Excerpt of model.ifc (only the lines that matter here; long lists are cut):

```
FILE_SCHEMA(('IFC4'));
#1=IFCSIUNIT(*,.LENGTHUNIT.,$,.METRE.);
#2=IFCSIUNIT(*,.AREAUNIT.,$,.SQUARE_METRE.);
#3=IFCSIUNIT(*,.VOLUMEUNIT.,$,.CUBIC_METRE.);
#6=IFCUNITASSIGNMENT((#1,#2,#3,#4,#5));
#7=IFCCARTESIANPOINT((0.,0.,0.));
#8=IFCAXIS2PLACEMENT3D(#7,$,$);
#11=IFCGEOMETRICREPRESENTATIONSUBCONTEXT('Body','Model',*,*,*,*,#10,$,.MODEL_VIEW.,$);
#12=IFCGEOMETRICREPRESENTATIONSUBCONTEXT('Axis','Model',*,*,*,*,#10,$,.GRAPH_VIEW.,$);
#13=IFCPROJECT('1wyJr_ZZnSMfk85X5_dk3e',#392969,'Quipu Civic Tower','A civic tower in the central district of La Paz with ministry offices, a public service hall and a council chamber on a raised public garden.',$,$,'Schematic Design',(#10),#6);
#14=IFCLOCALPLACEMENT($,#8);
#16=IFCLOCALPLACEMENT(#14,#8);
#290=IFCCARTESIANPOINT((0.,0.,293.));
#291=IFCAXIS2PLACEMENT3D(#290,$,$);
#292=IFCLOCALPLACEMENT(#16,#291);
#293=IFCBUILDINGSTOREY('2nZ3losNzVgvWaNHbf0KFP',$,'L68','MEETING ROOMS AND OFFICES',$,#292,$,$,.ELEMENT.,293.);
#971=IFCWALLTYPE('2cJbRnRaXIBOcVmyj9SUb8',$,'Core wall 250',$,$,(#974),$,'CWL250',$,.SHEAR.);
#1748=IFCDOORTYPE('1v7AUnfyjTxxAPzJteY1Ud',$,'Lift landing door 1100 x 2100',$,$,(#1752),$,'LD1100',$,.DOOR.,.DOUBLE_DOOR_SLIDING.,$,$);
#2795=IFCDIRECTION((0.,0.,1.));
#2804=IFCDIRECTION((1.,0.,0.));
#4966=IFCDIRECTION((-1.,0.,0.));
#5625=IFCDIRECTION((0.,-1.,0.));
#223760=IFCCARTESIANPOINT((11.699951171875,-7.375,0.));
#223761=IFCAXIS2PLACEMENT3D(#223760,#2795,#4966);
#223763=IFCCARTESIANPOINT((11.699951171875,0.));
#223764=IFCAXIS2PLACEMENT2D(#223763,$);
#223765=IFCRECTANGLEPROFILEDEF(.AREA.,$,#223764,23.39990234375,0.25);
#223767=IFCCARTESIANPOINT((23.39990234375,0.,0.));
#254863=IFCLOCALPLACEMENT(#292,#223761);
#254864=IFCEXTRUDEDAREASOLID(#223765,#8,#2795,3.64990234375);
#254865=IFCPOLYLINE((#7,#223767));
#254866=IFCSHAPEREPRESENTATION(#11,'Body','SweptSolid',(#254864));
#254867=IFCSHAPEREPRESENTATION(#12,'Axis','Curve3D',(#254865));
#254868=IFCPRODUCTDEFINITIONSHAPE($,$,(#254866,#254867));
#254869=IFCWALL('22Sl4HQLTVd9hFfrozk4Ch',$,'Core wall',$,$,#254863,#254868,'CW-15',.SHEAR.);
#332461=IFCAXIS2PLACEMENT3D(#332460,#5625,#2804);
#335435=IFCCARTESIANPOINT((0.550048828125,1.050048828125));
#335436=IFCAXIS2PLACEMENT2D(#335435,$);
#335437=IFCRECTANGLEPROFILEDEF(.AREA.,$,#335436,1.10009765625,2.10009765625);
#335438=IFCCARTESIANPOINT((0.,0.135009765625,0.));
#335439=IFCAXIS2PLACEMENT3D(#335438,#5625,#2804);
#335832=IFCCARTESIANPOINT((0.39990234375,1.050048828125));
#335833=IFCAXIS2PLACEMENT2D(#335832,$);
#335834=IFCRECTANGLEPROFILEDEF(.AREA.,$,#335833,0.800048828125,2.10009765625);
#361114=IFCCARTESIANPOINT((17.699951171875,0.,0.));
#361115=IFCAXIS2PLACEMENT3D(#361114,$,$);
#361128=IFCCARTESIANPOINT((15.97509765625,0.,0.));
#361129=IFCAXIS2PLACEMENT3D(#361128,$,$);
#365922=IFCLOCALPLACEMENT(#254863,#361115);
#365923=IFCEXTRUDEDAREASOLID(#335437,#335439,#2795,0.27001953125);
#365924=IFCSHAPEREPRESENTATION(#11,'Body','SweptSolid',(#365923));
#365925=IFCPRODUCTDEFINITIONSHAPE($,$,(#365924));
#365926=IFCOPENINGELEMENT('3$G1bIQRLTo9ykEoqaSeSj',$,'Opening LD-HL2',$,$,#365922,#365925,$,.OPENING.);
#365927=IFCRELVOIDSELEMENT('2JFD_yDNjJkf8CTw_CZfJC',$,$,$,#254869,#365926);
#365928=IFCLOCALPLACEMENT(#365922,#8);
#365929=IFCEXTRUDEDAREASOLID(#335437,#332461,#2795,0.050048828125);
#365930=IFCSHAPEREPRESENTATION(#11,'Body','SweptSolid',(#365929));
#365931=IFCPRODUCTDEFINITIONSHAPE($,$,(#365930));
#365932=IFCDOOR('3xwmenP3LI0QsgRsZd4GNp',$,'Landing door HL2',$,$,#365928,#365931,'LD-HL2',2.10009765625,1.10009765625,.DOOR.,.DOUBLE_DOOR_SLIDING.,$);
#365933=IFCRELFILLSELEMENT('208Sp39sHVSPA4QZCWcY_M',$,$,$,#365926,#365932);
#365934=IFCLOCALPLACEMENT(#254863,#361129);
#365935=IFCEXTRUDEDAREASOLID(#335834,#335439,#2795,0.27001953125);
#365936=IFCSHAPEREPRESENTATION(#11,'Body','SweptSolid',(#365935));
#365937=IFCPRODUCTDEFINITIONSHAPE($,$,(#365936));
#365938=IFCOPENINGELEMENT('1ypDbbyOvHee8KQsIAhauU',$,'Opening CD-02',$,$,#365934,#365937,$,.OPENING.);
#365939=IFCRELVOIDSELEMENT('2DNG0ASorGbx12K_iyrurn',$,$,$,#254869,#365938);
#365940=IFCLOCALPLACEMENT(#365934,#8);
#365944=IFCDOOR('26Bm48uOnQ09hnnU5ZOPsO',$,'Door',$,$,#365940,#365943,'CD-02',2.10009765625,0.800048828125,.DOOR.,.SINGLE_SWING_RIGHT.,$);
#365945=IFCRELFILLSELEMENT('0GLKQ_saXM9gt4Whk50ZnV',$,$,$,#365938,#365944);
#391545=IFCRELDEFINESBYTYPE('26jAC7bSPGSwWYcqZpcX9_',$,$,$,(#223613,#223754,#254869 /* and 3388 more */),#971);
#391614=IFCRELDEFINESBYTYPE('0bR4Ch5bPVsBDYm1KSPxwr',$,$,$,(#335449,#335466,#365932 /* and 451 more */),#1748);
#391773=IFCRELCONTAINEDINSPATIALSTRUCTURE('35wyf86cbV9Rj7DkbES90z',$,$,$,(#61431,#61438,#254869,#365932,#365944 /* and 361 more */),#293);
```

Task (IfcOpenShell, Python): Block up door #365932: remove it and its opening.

```python
import ifcopenshell
import ifcopenshell.api.feature
import ifcopenshell.api.root
import ifcopenshell.geom
import ifcopenshell.util.shape

model = ifcopenshell.open("model.ifc")
settings = ifcopenshell.geom.settings()


def volume(element):
    """Net volume in cubic metres, openings subtracted."""
    shape = ifcopenshell.geom.create_shape(settings, element)
    return ifcopenshell.util.shape.get_volume(shape.geometry)


door = model.by_guid("3xwmenP3LI0QsgRsZd4GNp")
opening = door.FillsVoids[0].RelatingOpeningElement
wall = opening.VoidsElements[0].RelatingBuildingElement
before = volume(wall)

ifcopenshell.api.root.remove_product(model, product=door)
ifcopenshell.api.feature.remove_feature(model, feature=opening)

after = volume(wall)

print(f"wall volume {before:.3f} -> {after:.3f} m3")

model.write("model_edited.ifc")
```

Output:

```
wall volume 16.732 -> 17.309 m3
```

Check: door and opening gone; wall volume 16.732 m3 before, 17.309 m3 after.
